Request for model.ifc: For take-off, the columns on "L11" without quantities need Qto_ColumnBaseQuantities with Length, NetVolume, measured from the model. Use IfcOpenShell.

First a look at what the model holds.

```python
import ifcopenshell
import ifcopenshell.util.element
import ifcopenshell.util.unit

model = ifcopenshell.open("model.ifc")
print(model.schema)
for unit_type in ("LENGTHUNIT", "AREAUNIT", "VOLUMEUNIT"):
    print(unit_type, ifcopenshell.util.unit.calculate_unit_scale(model, unit_type))
storey = next(s for s in model.by_type("IfcBuildingStorey") if s.Name == "L11")
columns = [e for e in ifcopenshell.util.element.get_decomposition(storey) if e.is_a("IfcColumn")]
for e in sorted(columns, key=lambda e: e.id()):
    print(e.id(), e.is_a(), e.Name, list(ifcopenshell.util.element.get_psets(e, qtos_only=True)), sep=" | ")
```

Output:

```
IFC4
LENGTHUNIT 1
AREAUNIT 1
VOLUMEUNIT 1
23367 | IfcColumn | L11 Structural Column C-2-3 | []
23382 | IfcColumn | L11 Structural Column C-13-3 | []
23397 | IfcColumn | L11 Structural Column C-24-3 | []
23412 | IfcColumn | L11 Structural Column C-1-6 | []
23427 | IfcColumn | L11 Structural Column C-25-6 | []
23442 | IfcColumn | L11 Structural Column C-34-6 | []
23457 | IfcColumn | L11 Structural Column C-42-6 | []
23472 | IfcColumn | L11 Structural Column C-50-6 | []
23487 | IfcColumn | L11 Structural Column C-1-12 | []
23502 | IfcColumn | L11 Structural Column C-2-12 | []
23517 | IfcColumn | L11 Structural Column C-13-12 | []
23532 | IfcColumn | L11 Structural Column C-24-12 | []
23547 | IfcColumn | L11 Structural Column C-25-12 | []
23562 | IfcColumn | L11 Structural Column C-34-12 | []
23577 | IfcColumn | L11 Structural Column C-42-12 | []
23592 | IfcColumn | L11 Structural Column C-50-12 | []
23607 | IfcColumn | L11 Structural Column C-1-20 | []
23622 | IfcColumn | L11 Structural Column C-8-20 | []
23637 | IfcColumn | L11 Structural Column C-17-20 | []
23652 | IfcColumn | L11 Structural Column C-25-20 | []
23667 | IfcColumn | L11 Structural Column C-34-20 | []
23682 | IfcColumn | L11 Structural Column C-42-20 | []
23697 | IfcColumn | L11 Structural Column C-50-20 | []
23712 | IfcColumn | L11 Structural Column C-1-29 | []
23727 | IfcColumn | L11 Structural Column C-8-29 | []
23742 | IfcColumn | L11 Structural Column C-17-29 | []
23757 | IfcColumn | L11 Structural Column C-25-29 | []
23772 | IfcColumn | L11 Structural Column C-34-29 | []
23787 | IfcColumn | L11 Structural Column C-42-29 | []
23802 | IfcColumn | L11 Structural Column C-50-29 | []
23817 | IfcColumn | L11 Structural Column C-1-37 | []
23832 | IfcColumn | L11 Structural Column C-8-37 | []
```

```python
import ifcopenshell
import ifcopenshell.api.pset
import ifcopenshell.geom
import ifcopenshell.util.element
import ifcopenshell.util.shape
import ifcopenshell.util.unit

model = ifcopenshell.open("model.ifc")
unit_scale = ifcopenshell.util.unit.calculate_unit_scale(model)
volume_scale = ifcopenshell.util.unit.calculate_unit_scale(model, "VOLUMEUNIT")
settings = ifcopenshell.geom.settings()

storey = next(s for s in model.by_type("IfcBuildingStorey") if s.Name == "L11")
columns = [e for e in ifcopenshell.util.element.get_decomposition(storey) if e.is_a("IfcColumn")]

for e in sorted(columns, key=lambda e: e.id()):
    if ifcopenshell.util.element.get_psets(e, qtos_only=True, should_inherit=False):
        continue
    # Geometry comes back in metres, in the element's own axes.
    shape = ifcopenshell.geom.create_shape(settings, e)
    values = {
        "Length": ifcopenshell.util.shape.get_z(shape.geometry) / unit_scale,
        "NetVolume": ifcopenshell.util.shape.get_volume(shape.geometry) / volume_scale,
    }
    qto = ifcopenshell.api.pset.add_qto(model, product=e, name="Qto_ColumnBaseQuantities")
    ifcopenshell.api.pset.edit_qto(model, qto=qto, properties=values)
    print(e.id(), {k: round(v, 3) for k, v in values.items()})

model.write("model_rev.ifc")
```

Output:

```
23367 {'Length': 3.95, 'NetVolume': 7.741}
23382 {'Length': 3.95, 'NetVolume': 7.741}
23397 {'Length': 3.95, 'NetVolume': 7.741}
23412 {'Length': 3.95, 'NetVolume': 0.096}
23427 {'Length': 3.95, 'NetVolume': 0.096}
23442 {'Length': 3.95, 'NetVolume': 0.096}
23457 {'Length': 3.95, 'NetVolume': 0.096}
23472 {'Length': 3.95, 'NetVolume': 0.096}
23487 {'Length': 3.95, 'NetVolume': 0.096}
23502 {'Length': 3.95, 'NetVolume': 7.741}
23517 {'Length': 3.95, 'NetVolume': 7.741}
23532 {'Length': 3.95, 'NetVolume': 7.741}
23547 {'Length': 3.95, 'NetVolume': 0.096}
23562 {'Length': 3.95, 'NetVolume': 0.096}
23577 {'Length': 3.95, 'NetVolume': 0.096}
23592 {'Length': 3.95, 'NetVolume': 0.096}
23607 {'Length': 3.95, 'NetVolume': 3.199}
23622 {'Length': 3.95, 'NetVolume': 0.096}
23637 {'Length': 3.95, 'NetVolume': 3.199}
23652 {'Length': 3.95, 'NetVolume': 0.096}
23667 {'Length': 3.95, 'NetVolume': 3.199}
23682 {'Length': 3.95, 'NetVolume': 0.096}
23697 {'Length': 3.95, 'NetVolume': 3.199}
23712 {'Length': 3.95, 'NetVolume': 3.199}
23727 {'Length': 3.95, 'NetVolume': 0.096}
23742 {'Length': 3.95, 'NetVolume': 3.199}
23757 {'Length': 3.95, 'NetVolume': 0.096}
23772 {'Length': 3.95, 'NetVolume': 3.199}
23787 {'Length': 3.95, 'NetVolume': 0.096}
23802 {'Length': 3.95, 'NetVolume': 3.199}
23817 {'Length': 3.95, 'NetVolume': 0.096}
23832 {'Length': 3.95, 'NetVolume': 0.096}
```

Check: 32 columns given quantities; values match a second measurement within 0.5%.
